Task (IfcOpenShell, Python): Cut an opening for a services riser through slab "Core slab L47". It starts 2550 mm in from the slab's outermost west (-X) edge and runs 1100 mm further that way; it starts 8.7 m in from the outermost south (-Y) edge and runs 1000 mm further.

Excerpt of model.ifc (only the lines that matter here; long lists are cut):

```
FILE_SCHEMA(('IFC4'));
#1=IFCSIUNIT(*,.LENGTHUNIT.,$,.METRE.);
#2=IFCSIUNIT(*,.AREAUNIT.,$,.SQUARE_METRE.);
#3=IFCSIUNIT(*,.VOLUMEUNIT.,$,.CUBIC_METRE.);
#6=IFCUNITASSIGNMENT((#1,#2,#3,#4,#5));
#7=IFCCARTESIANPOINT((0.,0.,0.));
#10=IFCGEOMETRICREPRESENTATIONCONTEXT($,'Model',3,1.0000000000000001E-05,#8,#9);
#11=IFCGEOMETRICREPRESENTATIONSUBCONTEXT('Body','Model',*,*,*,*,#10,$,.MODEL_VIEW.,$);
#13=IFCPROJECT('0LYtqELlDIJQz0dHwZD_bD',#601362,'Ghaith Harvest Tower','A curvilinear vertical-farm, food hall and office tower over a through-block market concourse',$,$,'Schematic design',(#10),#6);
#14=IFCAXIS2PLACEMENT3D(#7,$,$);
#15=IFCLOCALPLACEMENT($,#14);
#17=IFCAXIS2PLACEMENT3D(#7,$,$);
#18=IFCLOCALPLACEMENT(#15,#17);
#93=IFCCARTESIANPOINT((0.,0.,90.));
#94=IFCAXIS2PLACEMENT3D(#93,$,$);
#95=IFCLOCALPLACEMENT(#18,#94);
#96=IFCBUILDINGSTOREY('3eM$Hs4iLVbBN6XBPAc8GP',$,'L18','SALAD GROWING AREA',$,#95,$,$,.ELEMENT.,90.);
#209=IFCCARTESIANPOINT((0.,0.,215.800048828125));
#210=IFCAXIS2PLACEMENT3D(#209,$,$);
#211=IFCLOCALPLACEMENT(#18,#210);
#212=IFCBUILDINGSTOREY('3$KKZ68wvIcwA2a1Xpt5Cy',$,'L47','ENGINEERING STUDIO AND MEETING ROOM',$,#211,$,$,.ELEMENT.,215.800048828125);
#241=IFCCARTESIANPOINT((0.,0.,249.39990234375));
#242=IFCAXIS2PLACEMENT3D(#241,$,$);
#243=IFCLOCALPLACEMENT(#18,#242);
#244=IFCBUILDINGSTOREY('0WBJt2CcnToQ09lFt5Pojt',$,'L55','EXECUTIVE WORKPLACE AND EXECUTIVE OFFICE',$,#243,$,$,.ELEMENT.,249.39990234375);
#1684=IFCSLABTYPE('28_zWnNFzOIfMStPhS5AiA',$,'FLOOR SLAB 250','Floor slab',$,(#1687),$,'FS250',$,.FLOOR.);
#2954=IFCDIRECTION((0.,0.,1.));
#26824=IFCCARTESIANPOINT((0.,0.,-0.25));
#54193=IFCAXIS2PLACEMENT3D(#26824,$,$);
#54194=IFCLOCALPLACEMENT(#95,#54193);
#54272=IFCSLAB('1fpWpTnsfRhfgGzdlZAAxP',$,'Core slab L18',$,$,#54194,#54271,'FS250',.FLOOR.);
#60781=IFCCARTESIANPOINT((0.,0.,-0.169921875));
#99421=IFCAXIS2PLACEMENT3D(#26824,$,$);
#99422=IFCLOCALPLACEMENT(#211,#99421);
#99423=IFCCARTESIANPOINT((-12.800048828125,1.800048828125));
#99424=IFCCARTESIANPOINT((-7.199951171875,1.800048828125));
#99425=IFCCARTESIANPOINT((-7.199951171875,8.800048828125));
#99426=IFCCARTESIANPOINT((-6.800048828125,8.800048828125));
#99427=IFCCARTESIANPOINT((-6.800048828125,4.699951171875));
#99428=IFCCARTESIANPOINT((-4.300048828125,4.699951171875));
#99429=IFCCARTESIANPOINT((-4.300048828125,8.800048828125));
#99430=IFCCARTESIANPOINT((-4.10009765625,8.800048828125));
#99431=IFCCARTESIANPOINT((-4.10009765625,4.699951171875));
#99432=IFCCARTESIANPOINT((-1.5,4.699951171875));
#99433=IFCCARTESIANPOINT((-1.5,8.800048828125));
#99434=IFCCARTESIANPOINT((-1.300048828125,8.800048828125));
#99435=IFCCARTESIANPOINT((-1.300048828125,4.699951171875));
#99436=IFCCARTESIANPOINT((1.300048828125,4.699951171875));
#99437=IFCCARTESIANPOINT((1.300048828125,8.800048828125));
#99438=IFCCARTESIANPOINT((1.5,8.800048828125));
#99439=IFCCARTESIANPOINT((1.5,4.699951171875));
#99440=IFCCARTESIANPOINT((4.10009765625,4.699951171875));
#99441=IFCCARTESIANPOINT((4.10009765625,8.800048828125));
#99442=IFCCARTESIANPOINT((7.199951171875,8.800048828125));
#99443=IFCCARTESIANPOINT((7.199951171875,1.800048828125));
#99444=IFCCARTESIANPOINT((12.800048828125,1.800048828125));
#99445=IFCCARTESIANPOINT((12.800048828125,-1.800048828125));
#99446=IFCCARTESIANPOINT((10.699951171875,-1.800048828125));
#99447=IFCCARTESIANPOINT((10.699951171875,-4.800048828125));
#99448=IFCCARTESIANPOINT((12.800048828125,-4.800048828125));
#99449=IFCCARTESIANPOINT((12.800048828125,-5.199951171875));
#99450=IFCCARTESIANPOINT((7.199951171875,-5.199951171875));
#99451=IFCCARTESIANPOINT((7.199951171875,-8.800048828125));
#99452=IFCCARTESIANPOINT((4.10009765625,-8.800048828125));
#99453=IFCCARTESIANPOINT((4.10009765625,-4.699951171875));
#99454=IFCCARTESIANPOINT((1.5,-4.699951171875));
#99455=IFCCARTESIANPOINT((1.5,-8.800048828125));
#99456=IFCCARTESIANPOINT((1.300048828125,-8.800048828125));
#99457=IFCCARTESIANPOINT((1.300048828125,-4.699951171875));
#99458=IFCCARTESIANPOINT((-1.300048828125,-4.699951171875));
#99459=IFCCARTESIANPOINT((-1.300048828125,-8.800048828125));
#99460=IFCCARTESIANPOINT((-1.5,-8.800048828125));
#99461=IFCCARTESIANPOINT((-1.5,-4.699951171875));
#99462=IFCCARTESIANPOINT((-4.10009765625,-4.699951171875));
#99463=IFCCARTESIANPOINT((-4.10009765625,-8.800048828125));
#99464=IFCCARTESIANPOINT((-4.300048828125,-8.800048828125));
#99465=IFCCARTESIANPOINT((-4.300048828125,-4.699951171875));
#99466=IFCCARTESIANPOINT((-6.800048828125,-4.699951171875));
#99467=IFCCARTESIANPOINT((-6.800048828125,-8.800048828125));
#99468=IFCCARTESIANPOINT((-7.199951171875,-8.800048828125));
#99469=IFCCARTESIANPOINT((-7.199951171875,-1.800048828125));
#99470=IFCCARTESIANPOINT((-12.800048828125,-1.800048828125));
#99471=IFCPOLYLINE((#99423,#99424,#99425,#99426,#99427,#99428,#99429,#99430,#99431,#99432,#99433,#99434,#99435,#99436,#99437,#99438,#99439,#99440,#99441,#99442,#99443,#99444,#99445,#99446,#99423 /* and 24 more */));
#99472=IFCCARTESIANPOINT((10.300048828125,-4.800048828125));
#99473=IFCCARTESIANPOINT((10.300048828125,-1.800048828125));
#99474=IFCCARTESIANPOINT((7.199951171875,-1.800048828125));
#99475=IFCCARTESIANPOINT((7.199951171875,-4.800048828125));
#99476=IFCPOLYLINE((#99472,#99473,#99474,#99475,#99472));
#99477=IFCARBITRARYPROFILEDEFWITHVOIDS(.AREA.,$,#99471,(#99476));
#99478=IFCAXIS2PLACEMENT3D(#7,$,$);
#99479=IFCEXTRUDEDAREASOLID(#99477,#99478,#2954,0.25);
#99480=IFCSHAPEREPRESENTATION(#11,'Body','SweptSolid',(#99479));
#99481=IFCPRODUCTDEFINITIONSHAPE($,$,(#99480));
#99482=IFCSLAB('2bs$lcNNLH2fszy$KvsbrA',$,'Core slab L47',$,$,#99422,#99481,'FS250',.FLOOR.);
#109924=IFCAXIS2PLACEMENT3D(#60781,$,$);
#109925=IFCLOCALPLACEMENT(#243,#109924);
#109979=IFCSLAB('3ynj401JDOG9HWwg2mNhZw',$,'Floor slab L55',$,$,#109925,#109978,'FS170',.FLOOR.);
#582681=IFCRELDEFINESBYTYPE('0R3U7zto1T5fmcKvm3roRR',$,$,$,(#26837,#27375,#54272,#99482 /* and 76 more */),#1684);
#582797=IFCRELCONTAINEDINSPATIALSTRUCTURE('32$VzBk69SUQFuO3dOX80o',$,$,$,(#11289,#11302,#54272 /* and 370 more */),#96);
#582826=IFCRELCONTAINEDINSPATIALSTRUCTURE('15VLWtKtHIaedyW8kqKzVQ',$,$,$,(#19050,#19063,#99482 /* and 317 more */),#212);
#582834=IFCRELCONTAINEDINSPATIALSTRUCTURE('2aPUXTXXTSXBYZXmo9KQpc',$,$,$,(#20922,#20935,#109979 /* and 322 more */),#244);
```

```python
import numpy as np
import ifcopenshell
import ifcopenshell.api.feature
import ifcopenshell.api.geometry
import ifcopenshell.api.root
import ifcopenshell.geom
import ifcopenshell.util.placement
import ifcopenshell.util.representation
import ifcopenshell.util.shape
import ifcopenshell.util.unit

model = ifcopenshell.open("model.ifc")
unit_scale = ifcopenshell.util.unit.calculate_unit_scale(model)
settings = ifcopenshell.geom.settings()


def volume(element):
    """Net volume in cubic metres, openings subtracted."""
    shape = ifcopenshell.geom.create_shape(settings, element)
    return ifcopenshell.util.shape.get_volume(shape.geometry)


slab = model.by_id(99482)
before = volume(slab)

# Extent in the slab's own axes, in metres. The edges named are its -X and -Y sides.
slab_shape = ifcopenshell.geom.create_shape(settings, slab)
vertices = ifcopenshell.util.shape.get_vertices(slab_shape.geometry)
x_min, y_min, bottom = vertices.min(axis=0)
top = vertices[:, 2].max()

opening = ifcopenshell.api.root.create_entity(model, ifc_class="IfcOpeningElement", name="Services riser opening", predefined_type="OPENING")
context = ifcopenshell.util.representation.get_context(model, "Model", "Body", "MODEL_VIEW")
width, depth = 1.1, 1
outline = [(0.0, 0.0), (width, 0.0), (width, depth), (0.0, depth), (0.0, 0.0)]
# Overshoot both faces by 50 mm so the cut is clean.
shape = ifcopenshell.api.geometry.add_slab_representation(
    model, context=context, depth=top - bottom + 0.1, polyline=outline
)
ifcopenshell.api.geometry.assign_representation(model, product=opening, representation=shape)

matrix = ifcopenshell.util.placement.get_local_placement(slab.ObjectPlacement)
matrix[:, 3] = matrix @ np.append(np.array([x_min + 2.55, y_min + 8.7, bottom - 0.05]) / unit_scale, 1.0)
ifcopenshell.api.geometry.edit_object_placement(model, product=opening, matrix=matrix, is_si=False)
ifcopenshell.api.feature.add_feature(model, feature=opening, element=slab)

after = volume(slab)

print(f"slab volume {before:.3f} -> {after:.3f} m3")

model.write("model_updated.ifc")
```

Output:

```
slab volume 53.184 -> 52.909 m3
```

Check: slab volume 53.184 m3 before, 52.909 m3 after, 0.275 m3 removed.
